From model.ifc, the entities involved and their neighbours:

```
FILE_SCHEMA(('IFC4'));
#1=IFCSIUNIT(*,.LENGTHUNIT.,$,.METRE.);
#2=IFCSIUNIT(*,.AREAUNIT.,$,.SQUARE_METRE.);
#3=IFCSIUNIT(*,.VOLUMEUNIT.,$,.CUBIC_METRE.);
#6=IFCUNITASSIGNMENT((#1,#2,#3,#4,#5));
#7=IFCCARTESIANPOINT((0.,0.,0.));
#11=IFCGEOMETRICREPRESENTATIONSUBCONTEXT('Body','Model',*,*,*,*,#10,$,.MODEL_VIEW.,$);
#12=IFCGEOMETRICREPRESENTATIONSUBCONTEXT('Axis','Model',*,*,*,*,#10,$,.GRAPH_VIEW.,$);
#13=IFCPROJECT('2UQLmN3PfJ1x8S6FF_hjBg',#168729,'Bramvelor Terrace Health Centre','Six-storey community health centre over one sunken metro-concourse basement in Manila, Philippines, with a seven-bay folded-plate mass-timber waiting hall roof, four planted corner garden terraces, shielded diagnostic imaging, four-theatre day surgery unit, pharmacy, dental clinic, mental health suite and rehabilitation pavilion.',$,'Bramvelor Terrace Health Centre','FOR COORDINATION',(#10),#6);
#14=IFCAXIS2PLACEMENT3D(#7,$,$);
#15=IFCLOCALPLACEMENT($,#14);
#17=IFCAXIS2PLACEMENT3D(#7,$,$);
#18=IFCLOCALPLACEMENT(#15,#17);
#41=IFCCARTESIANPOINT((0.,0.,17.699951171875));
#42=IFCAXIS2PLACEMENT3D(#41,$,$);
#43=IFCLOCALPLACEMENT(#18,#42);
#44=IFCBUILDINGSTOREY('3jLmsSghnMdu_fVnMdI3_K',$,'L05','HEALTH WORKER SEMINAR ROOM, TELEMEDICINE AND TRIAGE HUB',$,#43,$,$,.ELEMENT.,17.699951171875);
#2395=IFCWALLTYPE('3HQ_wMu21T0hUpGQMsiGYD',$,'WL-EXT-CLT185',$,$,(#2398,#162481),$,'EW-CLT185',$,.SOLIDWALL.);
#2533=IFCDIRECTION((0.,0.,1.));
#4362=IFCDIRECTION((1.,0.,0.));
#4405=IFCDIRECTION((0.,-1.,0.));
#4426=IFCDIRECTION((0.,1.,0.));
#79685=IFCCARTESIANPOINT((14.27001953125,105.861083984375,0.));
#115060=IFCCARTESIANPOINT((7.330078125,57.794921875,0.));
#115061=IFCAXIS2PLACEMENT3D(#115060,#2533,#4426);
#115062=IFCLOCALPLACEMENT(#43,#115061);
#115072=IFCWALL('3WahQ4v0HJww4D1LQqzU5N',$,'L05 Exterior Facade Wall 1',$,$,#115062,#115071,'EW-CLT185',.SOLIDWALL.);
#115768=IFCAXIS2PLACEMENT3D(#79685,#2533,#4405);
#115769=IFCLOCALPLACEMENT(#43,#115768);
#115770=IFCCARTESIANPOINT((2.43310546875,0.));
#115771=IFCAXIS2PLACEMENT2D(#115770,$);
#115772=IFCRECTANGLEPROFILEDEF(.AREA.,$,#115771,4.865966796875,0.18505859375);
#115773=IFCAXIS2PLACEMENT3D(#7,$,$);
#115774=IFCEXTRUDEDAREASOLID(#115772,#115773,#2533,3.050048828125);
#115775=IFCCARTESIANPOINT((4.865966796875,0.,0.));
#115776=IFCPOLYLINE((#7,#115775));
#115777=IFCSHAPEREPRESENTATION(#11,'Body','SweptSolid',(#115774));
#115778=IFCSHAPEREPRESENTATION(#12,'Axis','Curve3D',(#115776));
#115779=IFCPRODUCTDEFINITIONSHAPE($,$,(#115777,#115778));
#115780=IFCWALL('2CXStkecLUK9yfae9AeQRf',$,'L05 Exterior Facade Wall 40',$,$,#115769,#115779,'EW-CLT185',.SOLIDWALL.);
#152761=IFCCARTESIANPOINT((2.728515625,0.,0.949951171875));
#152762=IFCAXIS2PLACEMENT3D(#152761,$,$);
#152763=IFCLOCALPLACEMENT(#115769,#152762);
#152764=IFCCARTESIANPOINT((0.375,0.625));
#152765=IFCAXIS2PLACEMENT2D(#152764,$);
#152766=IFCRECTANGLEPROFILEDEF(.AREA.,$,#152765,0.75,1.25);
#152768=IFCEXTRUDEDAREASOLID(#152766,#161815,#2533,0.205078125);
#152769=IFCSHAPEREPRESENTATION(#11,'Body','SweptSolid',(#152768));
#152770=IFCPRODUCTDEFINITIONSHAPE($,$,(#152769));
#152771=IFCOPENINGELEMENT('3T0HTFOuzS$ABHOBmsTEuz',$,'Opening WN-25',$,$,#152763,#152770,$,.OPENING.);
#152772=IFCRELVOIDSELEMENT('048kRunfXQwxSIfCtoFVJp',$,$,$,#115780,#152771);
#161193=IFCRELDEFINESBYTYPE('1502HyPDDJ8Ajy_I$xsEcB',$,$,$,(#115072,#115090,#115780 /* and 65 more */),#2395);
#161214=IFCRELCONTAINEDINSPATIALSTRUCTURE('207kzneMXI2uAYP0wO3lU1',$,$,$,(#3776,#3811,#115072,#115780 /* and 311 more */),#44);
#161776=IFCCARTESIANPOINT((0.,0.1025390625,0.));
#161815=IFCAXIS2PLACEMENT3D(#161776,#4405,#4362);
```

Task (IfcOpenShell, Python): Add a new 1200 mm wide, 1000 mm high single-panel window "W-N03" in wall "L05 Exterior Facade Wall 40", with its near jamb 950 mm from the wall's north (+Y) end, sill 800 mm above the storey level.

```python
import numpy as np
import ifcopenshell
import ifcopenshell.api.feature
import ifcopenshell.api.geometry
import ifcopenshell.api.root
import ifcopenshell.api.spatial
import ifcopenshell.geom
import ifcopenshell.util.element
import ifcopenshell.util.placement
import ifcopenshell.util.representation
import ifcopenshell.util.shape
import ifcopenshell.util.unit

model = ifcopenshell.open("model.ifc")
unit_scale = ifcopenshell.util.unit.calculate_unit_scale(model)
settings = ifcopenshell.geom.settings()


def volume(element):
    """Net volume in cubic metres, openings subtracted."""
    shape = ifcopenshell.geom.create_shape(settings, element)
    return ifcopenshell.util.shape.get_volume(shape.geometry)


wall = model.by_guid("2CXStkecLUK9yfae9AeQRf")
storey = ifcopenshell.util.element.get_container(wall, ifc_class="IfcBuildingStorey")
context = ifcopenshell.util.representation.get_context(model, "Model", "Body", "MODEL_VIEW")
before = volume(wall)

width, height, from_end, sill = 1.2, 1, 0.95, 0.8  # metres

# The wall runs along its own X axis, and the end named is its -X end.
wall_shape = ifcopenshell.geom.create_shape(settings, wall)
x, y, z = ifcopenshell.util.shape.get_vertices(wall_shape.geometry).T
start = x.min() + from_end
face, thickness = float(y.min()), float(y.max() - y.min())
wall_matrix = ifcopenshell.util.placement.get_local_placement(wall.ObjectPlacement)
level = ifcopenshell.util.placement.get_local_placement(storey.ObjectPlacement)[2, 3]


def in_wall(x, y):
    """Placement at x, y metres in the wall's axes, at sill height."""
    matrix = wall_matrix.copy()
    matrix[:, 3] = wall_matrix @ np.array([x / unit_scale, y / unit_scale, 0.0, 1.0])
    matrix[2, 3] = level + sill / unit_scale
    return matrix


# Opening: a box that overshoots both wall faces by 50 mm.
opening = ifcopenshell.api.root.create_entity(model, ifc_class="IfcOpeningElement", predefined_type="OPENING")
box = ifcopenshell.api.geometry.add_wall_representation(
    model, context=context, length=width, height=height, thickness=thickness + 0.1
)
ifcopenshell.api.geometry.assign_representation(model, product=opening, representation=box)
ifcopenshell.api.geometry.edit_object_placement(model, product=opening, matrix=in_wall(start, face - 0.05), is_si=False)
ifcopenshell.api.feature.add_feature(model, feature=opening, element=wall)

window = ifcopenshell.api.root.create_entity(model, ifc_class="IfcWindow", name="W-N03", predefined_type="WINDOW")
window.OverallWidth, window.OverallHeight = width / unit_scale, height / unit_scale
window.PartitioningType = "SINGLE_PANEL"
body = ifcopenshell.api.geometry.add_window_representation(
    model,
    context=context,
    overall_width=window.OverallWidth,
    overall_height=window.OverallHeight,
    partition_type="SINGLE_PANEL",
)
ifcopenshell.api.geometry.assign_representation(model, product=window, representation=body)
ifcopenshell.api.spatial.assign_container(model, products=[window], relating_structure=storey)
ifcopenshell.api.feature.add_filling(model, opening=opening, element=window)

# Centre the window in the wall's thickness.
ifcopenshell.api.geometry.edit_object_placement(model, product=window, matrix=in_wall(start, face), is_si=False)
window_shape = ifcopenshell.geom.create_shape(settings, window)
depth = ifcopenshell.util.shape.get_vertices(window_shape.geometry)[:, 1]
offset = face + thickness / 2 - (depth.min() + depth.max()) / 2
ifcopenshell.api.geometry.edit_object_placement(model, product=window, matrix=in_wall(start, offset), is_si=False)

after = volume(wall)

print(f"wall volume {before:.3f} -> {after:.3f} m3")

model.write("model-out.ifc")
```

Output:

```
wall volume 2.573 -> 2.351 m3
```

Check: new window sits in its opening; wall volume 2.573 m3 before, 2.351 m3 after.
